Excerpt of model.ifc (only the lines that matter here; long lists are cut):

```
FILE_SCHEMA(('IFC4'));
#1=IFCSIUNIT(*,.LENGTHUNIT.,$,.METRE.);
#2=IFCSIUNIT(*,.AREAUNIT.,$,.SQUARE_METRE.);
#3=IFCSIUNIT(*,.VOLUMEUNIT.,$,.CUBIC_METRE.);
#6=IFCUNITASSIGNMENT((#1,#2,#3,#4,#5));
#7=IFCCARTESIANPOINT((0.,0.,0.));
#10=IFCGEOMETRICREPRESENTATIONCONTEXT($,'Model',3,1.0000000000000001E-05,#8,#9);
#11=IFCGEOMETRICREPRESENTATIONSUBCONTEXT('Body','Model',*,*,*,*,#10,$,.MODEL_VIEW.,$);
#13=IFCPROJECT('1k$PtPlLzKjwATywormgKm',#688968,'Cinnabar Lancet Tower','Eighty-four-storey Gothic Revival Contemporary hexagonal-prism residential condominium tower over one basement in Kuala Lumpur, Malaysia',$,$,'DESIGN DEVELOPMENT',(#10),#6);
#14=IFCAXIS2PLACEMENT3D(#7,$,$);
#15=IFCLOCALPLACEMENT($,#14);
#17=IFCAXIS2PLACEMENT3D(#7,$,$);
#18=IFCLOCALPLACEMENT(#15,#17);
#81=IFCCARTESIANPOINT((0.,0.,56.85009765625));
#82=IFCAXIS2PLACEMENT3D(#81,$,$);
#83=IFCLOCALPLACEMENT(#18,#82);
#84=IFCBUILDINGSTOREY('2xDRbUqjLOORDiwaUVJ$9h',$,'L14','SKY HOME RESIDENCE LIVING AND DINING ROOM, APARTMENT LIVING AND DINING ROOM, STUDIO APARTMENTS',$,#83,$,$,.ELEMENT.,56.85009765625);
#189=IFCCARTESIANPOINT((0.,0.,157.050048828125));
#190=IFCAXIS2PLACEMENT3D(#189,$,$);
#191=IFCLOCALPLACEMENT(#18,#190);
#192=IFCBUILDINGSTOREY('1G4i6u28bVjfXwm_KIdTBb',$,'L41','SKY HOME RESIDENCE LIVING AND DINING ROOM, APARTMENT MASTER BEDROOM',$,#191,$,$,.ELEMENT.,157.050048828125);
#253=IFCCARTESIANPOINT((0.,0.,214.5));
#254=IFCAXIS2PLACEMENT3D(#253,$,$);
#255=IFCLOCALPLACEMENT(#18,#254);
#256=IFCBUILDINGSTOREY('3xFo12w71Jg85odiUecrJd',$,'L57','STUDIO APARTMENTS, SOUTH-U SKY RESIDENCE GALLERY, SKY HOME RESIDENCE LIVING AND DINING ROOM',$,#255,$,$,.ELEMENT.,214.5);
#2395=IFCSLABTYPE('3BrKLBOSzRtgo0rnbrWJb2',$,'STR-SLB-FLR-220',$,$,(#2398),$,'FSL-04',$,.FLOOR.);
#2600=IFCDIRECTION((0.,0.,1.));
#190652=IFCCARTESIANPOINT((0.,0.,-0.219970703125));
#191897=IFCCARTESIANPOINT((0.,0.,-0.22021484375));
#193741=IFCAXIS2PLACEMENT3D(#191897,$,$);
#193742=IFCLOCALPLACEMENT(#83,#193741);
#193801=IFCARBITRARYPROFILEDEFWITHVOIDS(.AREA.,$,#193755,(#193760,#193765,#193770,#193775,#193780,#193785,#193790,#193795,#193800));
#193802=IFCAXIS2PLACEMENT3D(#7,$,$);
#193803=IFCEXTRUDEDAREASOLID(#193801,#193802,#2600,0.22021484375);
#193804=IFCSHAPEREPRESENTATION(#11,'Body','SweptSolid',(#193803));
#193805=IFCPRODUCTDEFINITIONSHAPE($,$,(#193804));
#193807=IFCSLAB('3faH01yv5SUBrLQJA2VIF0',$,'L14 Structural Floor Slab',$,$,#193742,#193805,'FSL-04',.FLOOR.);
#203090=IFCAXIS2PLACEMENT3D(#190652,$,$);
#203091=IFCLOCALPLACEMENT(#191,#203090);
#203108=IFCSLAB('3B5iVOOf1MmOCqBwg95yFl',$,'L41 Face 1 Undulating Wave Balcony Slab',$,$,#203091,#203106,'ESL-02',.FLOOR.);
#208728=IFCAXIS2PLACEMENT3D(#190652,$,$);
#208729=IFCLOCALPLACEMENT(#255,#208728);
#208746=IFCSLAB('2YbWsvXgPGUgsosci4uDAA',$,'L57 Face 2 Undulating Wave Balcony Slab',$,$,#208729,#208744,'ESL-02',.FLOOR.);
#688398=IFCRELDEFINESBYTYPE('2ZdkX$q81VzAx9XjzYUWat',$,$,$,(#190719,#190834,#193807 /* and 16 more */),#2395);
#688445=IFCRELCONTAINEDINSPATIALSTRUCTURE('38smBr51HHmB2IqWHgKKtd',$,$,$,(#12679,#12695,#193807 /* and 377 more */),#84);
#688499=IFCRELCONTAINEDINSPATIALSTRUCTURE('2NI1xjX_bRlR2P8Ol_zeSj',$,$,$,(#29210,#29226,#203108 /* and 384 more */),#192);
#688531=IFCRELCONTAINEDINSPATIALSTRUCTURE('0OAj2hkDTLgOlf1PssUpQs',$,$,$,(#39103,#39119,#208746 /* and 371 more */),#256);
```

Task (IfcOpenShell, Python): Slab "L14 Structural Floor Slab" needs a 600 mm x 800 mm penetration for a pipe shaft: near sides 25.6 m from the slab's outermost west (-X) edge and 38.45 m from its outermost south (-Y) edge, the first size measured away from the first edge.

```python
import numpy as np
import ifcopenshell
import ifcopenshell.api.feature
import ifcopenshell.api.geometry
import ifcopenshell.api.root
import ifcopenshell.geom
import ifcopenshell.util.placement
import ifcopenshell.util.representation
import ifcopenshell.util.shape
import ifcopenshell.util.unit

model = ifcopenshell.open("model.ifc")
unit_scale = ifcopenshell.util.unit.calculate_unit_scale(model)
settings = ifcopenshell.geom.settings()


def volume(element):
    """Net volume in cubic metres, openings subtracted."""
    shape = ifcopenshell.geom.create_shape(settings, element)
    return ifcopenshell.util.shape.get_volume(shape.geometry)


slab = model.by_guid("3faH01yv5SUBrLQJA2VIF0")
before = volume(slab)

# Extent in the slab's own axes, in metres. The edges named are its -X and -Y sides.
slab_shape = ifcopenshell.geom.create_shape(settings, slab)
vertices = ifcopenshell.util.shape.get_vertices(slab_shape.geometry)
x_min, y_min, bottom = vertices.min(axis=0)
top = vertices[:, 2].max()

opening = ifcopenshell.api.root.create_entity(model, ifc_class="IfcOpeningElement", name="Pipe shaft opening", predefined_type="OPENING")
context = ifcopenshell.util.representation.get_context(model, "Model", "Body", "MODEL_VIEW")
width, depth = 0.6, 0.8
outline = [(0.0, 0.0), (width, 0.0), (width, depth), (0.0, depth), (0.0, 0.0)]
# Overshoot both faces by 50 mm so the cut is clean.
shape = ifcopenshell.api.geometry.add_slab_representation(
    model, context=context, depth=top - bottom + 0.1, polyline=outline
)
ifcopenshell.api.geometry.assign_representation(model, product=opening, representation=shape)

matrix = ifcopenshell.util.placement.get_local_placement(slab.ObjectPlacement)
matrix[:, 3] = matrix @ np.append(np.array([x_min + 25.6, y_min + 38.45, bottom - 0.05]) / unit_scale, 1.0)
ifcopenshell.api.geometry.edit_object_placement(model, product=opening, matrix=matrix, is_si=False)
ifcopenshell.api.feature.add_feature(model, feature=opening, element=slab)

after = volume(slab)

print(f"slab volume {before:.3f} -> {after:.3f} m3")

model.write("model_edited.ifc")
```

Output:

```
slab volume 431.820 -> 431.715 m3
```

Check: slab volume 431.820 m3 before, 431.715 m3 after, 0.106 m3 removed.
